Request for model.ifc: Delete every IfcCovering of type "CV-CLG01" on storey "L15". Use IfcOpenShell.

First a look at what the model holds.

```python
import ifcopenshell
import ifcopenshell.util.element

model = ifcopenshell.open("model.ifc")
print(model.schema)
storey = next(s for s in model.by_type("IfcBuildingStorey") if s.Name == "L15")
coverings = [e for e in ifcopenshell.util.element.get_decomposition(storey) if e.is_a("IfcCovering")]
seen = {}
for e in coverings:
    element_type = ifcopenshell.util.element.get_type(e)
    name = element_type.Name if element_type not in (None, e) else None
    seen[name] = seen.get(name, 0) + 1
for name, count in sorted(seen.items(), key=str):
    print(count, "x", name)
```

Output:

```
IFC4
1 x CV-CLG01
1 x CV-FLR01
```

```python
import ifcopenshell
import ifcopenshell.api.root
import ifcopenshell.util.element

model = ifcopenshell.open("model.ifc")

storey = next(s for s in model.by_type("IfcBuildingStorey") if s.Name == "L15")
coverings = [e for e in ifcopenshell.util.element.get_decomposition(storey) if e.is_a("IfcCovering")]
targets = [e for e in coverings if (t := ifcopenshell.util.element.get_type(e)) not in (None, e) and t.Name == "CV-CLG01"]

for e in targets:
    ifcopenshell.api.root.remove_product(model, product=e)
print(len(targets), "removed")

model.write("model-out.ifc")
```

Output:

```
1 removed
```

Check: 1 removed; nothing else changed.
